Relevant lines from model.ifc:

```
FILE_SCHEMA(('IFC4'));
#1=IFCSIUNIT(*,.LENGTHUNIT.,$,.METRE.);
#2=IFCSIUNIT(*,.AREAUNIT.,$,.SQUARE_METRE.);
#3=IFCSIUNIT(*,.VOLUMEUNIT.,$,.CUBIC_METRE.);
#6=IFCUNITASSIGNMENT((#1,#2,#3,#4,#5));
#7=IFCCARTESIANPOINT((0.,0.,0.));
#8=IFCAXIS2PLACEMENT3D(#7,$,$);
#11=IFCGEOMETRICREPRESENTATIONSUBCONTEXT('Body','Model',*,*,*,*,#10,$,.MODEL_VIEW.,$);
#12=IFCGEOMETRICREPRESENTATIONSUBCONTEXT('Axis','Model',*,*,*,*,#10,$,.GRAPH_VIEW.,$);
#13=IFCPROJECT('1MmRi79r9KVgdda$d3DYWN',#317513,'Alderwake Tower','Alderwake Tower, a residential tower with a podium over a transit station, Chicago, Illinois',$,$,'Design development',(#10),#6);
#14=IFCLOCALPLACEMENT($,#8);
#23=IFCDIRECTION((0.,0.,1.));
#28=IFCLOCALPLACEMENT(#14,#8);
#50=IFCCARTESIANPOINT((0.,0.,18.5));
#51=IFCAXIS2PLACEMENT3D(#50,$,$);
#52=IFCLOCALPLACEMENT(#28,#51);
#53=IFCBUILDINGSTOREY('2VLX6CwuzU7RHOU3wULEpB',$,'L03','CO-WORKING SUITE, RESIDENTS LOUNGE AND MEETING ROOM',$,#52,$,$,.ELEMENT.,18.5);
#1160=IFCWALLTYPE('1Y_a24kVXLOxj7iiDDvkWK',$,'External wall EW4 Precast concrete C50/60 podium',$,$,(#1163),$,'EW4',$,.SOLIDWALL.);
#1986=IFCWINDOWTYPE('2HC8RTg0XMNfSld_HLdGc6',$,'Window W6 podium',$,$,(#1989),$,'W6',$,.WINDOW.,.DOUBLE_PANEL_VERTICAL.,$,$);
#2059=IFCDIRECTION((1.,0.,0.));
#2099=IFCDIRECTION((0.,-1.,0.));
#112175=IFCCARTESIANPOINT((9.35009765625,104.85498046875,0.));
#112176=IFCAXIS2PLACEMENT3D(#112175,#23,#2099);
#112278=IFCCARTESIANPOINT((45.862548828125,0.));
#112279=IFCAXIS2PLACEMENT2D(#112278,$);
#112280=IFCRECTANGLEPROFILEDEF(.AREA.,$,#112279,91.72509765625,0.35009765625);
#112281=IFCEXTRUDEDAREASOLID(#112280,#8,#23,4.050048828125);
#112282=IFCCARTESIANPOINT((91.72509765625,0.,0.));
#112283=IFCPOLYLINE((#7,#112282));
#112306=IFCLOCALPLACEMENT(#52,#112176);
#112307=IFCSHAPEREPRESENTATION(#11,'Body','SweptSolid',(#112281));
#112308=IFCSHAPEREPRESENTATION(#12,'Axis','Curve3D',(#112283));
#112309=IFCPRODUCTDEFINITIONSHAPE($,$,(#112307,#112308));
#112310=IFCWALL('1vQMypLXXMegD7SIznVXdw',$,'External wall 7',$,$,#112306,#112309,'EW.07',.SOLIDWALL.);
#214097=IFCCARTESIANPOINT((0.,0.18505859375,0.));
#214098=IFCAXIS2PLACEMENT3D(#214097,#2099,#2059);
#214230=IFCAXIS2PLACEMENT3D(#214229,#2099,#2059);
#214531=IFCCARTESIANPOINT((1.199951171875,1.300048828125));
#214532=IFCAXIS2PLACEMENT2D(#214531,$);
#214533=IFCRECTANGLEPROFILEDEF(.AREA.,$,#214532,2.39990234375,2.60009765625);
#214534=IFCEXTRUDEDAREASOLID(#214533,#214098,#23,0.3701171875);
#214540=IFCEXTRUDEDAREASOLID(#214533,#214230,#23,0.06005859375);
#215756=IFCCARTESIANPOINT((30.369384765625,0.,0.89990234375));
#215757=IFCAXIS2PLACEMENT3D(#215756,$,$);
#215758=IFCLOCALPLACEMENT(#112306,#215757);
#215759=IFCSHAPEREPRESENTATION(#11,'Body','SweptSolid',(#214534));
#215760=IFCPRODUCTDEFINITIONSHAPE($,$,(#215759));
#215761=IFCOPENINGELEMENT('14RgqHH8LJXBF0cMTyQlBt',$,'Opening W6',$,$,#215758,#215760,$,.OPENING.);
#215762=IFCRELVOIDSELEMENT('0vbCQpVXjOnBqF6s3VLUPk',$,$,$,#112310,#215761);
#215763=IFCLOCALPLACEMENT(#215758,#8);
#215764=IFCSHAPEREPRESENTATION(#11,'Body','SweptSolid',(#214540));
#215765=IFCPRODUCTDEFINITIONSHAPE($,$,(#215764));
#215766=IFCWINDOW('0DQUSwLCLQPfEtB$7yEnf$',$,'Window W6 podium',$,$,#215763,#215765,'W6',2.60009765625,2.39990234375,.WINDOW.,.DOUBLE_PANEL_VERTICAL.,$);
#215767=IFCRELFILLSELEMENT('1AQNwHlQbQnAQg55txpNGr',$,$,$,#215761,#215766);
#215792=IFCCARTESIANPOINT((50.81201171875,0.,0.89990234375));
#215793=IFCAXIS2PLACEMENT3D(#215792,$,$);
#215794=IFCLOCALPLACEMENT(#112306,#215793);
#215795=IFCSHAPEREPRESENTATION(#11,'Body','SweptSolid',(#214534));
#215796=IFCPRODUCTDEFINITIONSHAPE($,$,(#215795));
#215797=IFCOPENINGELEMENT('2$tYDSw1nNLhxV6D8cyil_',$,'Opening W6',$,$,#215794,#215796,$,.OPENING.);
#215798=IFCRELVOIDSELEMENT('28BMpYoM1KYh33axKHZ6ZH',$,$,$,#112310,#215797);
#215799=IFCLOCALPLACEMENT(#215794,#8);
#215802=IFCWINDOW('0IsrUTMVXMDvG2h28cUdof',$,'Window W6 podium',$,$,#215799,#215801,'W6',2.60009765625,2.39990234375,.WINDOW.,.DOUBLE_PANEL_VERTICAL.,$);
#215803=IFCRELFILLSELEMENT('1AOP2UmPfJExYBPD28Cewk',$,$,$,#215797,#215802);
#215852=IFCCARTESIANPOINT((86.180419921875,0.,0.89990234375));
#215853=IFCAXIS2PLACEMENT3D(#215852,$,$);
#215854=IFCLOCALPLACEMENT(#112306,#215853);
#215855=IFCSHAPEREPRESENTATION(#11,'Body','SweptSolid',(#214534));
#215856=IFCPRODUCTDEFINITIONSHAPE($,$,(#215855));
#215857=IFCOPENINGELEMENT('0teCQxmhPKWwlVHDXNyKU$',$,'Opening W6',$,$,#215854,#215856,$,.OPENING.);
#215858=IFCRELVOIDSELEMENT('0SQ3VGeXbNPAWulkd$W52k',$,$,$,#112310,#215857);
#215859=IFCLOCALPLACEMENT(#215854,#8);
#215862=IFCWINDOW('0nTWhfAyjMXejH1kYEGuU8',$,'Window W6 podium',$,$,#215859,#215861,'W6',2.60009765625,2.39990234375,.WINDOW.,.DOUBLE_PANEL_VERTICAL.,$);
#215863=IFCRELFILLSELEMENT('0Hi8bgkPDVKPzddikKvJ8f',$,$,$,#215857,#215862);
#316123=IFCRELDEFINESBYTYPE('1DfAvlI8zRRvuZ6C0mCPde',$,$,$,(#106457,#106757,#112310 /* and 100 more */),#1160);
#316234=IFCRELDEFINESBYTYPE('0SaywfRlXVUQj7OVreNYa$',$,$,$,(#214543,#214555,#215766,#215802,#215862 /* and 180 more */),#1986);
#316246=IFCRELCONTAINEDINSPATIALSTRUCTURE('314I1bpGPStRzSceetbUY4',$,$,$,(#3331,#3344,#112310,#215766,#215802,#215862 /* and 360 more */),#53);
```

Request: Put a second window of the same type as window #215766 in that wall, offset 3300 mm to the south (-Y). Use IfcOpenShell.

```python
import ifcopenshell
import ifcopenshell.api.feature
import ifcopenshell.api.geometry
import ifcopenshell.api.root
import ifcopenshell.geom
import ifcopenshell.util.element
import ifcopenshell.util.placement
import ifcopenshell.util.shape

model = ifcopenshell.open("model.ifc")
settings = ifcopenshell.geom.settings()


def volume(element):
    """Net volume in cubic metres, openings subtracted."""
    shape = ifcopenshell.geom.create_shape(settings, element)
    return ifcopenshell.util.shape.get_volume(shape.geometry)


window = model.by_guid("0DQUSwLCLQPfEtB$7yEnf$")
opening = window.FillsVoids[0].RelatingOpeningElement
wall = opening.VoidsElements[0].RelatingBuildingElement
before = volume(wall)
shift = ifcopenshell.util.placement.get_local_placement(wall.ObjectPlacement)[:3, 0] * 3.3

# copy_class copies the void relationship, type, container and properties, but no geometry.
new_opening = ifcopenshell.api.root.copy_class(model, product=opening)
new_opening.Representation = ifcopenshell.util.element.copy_deep(
    model, opening.Representation, exclude=["IfcGeometricRepresentationContext", "IfcRepresentationMap"]
)
new_window = ifcopenshell.api.root.copy_class(model, product=window)
new_window.Representation = ifcopenshell.util.element.copy_deep(
    model, window.Representation, exclude=["IfcGeometricRepresentationContext", "IfcRepresentationMap"]
)
new_window.Tag = None
ifcopenshell.api.feature.add_filling(model, opening=new_opening, element=new_window)

for old, new in ((opening, new_opening), (window, new_window)):
    matrix = ifcopenshell.util.placement.get_local_placement(old.ObjectPlacement)
    matrix[:3, 3] += shift
    ifcopenshell.api.geometry.edit_object_placement(model, product=new, matrix=matrix, is_si=False)

after = volume(wall)

print(f"wall volume {before:.3f} -> {after:.3f} m3")

model.write("model_v2.ifc")
```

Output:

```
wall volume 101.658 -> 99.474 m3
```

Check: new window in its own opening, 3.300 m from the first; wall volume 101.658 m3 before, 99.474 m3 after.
